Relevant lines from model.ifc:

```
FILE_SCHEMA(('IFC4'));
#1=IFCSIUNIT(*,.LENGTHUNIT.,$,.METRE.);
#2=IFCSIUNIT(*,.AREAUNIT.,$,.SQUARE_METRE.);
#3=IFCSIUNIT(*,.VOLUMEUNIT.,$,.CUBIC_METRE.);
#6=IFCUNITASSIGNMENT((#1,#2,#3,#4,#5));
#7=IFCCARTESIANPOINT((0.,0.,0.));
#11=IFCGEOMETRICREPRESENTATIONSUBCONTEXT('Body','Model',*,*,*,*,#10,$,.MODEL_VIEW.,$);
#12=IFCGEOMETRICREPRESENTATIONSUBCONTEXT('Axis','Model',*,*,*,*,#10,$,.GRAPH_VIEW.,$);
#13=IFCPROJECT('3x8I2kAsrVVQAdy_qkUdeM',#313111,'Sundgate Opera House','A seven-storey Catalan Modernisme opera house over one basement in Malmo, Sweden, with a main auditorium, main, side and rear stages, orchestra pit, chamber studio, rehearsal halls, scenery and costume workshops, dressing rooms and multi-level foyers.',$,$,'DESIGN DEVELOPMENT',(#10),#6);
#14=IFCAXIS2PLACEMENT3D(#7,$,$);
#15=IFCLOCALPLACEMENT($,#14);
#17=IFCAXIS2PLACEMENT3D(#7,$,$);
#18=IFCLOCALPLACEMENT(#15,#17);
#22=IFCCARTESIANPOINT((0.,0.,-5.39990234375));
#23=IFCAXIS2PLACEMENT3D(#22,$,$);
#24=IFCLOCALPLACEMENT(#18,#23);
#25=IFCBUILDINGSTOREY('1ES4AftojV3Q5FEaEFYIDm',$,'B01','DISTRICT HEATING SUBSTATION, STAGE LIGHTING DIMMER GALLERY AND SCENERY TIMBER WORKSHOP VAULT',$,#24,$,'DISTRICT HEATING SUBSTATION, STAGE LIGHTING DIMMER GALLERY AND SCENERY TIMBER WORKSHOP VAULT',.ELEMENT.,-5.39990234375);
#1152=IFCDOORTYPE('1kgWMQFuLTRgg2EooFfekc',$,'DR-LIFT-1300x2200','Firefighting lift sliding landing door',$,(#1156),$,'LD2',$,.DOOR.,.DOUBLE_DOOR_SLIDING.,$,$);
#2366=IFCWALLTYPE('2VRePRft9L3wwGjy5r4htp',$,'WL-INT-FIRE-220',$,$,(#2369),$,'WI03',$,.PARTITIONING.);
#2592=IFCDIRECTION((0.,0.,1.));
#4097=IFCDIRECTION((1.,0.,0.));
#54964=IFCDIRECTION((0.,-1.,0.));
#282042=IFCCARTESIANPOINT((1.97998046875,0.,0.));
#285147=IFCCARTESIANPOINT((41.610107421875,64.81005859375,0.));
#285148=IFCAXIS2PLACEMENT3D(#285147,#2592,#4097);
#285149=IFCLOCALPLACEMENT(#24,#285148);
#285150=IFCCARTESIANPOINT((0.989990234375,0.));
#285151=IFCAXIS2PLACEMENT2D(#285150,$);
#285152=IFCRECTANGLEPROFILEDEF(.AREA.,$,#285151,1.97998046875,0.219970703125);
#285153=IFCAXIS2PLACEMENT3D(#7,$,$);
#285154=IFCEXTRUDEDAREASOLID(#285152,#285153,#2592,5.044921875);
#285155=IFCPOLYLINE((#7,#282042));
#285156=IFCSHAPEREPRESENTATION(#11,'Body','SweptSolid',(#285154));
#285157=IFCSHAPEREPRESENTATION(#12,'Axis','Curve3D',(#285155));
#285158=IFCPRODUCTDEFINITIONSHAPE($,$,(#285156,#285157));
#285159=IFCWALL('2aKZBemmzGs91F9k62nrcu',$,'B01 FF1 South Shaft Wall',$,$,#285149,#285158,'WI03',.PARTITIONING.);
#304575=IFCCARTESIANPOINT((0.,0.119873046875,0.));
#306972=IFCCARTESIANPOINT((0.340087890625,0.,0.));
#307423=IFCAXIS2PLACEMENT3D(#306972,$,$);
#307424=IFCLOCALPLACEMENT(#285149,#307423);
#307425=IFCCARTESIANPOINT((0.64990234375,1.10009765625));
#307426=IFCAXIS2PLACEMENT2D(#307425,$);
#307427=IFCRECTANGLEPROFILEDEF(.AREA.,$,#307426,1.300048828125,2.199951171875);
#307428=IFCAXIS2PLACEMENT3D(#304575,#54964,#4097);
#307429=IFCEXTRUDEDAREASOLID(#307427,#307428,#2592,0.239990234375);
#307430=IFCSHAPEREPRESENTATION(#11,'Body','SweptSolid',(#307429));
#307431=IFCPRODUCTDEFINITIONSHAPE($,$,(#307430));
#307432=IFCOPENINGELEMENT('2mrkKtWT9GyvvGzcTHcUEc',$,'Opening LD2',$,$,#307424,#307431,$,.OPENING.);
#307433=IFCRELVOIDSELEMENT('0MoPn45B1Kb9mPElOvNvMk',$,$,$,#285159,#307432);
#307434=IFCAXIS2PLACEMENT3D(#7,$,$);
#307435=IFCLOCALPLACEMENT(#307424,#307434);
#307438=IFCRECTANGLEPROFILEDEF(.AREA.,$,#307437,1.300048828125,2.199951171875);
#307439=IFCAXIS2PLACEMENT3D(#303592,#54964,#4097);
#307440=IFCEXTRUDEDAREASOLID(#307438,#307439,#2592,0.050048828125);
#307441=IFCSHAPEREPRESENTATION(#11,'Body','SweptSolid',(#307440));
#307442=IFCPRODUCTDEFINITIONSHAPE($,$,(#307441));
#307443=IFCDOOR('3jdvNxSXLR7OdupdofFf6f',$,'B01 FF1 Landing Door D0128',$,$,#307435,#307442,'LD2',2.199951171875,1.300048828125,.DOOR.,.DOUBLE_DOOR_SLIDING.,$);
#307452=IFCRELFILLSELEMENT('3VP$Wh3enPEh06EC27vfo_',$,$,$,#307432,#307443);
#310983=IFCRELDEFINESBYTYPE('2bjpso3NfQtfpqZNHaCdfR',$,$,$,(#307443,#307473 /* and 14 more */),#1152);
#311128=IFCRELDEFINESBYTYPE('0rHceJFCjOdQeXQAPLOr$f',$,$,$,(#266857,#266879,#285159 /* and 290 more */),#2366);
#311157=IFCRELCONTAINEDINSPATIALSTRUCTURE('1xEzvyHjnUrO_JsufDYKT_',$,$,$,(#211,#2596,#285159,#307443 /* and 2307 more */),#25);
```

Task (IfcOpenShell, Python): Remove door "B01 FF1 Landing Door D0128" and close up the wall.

```python
import ifcopenshell
import ifcopenshell.api.feature
import ifcopenshell.api.root
import ifcopenshell.geom
import ifcopenshell.util.shape

model = ifcopenshell.open("model.ifc")
settings = ifcopenshell.geom.settings()


def volume(element):
    """Net volume in cubic metres, openings subtracted."""
    shape = ifcopenshell.geom.create_shape(settings, element)
    return ifcopenshell.util.shape.get_volume(shape.geometry)


door = model.by_id(307443)
opening = door.FillsVoids[0].RelatingOpeningElement
wall = opening.VoidsElements[0].RelatingBuildingElement
before = volume(wall)

ifcopenshell.api.root.remove_product(model, product=door)
ifcopenshell.api.feature.remove_feature(model, feature=opening)

after = volume(wall)

print(f"wall volume {before:.3f} -> {after:.3f} m3")

model.write("model_updated.ifc")
```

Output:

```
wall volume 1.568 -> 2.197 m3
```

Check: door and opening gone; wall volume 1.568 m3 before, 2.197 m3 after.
